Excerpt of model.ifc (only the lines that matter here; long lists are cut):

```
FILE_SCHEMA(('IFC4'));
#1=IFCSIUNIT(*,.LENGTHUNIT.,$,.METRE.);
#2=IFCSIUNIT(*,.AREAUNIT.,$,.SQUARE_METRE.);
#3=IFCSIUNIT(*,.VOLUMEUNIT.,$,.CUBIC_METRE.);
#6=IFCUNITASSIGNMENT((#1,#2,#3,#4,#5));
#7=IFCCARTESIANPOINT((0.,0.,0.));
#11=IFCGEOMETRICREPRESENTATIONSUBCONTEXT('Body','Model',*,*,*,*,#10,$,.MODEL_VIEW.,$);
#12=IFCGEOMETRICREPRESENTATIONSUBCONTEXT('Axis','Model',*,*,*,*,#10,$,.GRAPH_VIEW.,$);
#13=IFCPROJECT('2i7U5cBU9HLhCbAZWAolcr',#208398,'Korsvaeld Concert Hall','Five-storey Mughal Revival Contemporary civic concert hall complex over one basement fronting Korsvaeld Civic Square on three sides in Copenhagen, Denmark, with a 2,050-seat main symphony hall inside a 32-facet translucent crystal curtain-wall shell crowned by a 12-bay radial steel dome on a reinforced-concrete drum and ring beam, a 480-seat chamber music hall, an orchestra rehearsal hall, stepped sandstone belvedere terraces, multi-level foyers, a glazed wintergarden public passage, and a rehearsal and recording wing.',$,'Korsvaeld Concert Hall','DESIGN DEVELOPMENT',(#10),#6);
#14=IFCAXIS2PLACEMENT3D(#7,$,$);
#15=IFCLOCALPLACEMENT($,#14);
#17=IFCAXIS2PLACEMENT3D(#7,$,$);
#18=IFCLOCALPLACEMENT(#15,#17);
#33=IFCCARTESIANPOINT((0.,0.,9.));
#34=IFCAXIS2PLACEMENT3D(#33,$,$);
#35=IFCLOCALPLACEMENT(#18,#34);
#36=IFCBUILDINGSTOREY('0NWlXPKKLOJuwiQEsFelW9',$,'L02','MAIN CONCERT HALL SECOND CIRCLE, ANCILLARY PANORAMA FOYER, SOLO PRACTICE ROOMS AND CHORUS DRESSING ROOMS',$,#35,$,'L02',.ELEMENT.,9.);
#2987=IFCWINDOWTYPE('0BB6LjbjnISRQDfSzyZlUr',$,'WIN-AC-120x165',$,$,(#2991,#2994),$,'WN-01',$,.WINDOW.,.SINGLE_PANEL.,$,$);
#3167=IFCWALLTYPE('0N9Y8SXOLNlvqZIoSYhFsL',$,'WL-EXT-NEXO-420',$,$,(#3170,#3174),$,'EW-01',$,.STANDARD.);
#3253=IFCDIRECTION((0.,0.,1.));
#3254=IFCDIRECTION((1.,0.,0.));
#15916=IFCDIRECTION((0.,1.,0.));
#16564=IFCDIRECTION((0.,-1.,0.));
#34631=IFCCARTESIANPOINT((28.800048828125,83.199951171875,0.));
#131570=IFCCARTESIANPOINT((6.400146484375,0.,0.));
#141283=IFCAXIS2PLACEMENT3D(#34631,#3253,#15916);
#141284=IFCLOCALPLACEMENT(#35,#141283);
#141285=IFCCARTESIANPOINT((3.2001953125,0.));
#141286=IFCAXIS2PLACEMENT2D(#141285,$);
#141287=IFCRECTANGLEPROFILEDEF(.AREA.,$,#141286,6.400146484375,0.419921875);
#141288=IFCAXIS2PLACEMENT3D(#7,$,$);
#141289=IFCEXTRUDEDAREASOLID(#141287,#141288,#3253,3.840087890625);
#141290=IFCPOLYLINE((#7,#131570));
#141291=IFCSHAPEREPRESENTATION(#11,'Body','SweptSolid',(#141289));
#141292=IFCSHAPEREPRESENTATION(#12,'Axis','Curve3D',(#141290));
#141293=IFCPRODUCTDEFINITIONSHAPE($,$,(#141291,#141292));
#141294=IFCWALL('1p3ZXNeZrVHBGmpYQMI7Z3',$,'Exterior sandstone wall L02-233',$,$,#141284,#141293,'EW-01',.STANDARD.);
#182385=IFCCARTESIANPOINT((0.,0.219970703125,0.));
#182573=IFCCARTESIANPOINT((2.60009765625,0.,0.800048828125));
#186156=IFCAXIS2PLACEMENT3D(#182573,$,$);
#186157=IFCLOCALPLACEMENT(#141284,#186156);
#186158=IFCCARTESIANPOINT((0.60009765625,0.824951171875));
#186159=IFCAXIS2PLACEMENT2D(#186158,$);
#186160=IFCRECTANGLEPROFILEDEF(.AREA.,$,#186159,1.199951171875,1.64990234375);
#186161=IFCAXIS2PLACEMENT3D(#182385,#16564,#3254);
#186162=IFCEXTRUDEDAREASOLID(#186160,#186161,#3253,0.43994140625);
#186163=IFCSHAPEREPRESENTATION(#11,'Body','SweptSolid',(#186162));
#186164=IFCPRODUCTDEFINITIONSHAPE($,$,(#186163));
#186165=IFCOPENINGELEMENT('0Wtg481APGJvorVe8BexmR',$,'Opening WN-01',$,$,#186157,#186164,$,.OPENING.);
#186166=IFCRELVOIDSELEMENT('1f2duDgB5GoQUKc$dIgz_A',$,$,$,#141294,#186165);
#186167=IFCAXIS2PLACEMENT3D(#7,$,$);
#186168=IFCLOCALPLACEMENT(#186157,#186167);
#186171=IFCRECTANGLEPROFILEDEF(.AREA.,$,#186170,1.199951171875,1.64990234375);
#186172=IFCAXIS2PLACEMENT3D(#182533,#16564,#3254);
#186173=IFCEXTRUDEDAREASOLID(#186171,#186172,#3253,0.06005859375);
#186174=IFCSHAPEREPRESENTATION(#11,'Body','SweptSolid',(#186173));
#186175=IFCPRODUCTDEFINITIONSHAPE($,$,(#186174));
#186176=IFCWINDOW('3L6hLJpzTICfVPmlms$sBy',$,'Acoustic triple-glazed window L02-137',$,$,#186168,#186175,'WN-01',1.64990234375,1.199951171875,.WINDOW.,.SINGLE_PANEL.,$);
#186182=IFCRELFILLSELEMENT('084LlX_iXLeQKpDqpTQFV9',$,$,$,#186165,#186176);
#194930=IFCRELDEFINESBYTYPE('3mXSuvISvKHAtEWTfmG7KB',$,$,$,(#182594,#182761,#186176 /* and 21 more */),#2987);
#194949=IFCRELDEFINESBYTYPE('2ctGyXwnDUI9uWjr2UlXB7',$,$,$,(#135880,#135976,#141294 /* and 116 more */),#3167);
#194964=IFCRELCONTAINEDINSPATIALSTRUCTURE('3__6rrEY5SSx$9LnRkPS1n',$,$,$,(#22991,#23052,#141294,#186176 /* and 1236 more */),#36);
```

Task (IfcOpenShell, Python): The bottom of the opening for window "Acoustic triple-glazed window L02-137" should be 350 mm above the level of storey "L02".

```python
import numpy as np
import ifcopenshell
import ifcopenshell.api.geometry
import ifcopenshell.geom
import ifcopenshell.util.element
import ifcopenshell.util.placement
import ifcopenshell.util.shape
import ifcopenshell.util.unit

model = ifcopenshell.open("model.ifc")
unit_scale = ifcopenshell.util.unit.calculate_unit_scale(model)

window = model.by_guid("3L6hLJpzTICfVPmlms$sBy")
opening = window.FillsVoids[0].RelatingOpeningElement
storey = ifcopenshell.util.element.get_container(window, ifc_class="IfcBuildingStorey")
level = ifcopenshell.util.placement.get_local_placement(storey.ObjectPlacement)[2, 3]

# The opening's origin need not be at the sill, so measure its lowest point.
shape = ifcopenshell.geom.create_shape(ifcopenshell.geom.settings(), opening)
bottom = ifcopenshell.util.shape.get_shape_bottom_elevation(shape, shape.geometry) / unit_scale
dz = level + 0.35 / unit_scale - bottom

shift = np.array([0.0, 0.0, dz])
# The window is placed relative to its opening, so it follows when the opening moves.
matrix = ifcopenshell.util.placement.get_local_placement(opening.ObjectPlacement)
matrix[:3, 3] += shift
ifcopenshell.api.geometry.edit_object_placement(
    model, product=opening, matrix=matrix, is_si=False, should_transform_children=True
)

print(f"moved by {dz * unit_scale:+.3f} m")

model.write("model_updated.ifc")
```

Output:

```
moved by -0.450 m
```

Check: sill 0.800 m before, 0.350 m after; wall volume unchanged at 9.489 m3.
